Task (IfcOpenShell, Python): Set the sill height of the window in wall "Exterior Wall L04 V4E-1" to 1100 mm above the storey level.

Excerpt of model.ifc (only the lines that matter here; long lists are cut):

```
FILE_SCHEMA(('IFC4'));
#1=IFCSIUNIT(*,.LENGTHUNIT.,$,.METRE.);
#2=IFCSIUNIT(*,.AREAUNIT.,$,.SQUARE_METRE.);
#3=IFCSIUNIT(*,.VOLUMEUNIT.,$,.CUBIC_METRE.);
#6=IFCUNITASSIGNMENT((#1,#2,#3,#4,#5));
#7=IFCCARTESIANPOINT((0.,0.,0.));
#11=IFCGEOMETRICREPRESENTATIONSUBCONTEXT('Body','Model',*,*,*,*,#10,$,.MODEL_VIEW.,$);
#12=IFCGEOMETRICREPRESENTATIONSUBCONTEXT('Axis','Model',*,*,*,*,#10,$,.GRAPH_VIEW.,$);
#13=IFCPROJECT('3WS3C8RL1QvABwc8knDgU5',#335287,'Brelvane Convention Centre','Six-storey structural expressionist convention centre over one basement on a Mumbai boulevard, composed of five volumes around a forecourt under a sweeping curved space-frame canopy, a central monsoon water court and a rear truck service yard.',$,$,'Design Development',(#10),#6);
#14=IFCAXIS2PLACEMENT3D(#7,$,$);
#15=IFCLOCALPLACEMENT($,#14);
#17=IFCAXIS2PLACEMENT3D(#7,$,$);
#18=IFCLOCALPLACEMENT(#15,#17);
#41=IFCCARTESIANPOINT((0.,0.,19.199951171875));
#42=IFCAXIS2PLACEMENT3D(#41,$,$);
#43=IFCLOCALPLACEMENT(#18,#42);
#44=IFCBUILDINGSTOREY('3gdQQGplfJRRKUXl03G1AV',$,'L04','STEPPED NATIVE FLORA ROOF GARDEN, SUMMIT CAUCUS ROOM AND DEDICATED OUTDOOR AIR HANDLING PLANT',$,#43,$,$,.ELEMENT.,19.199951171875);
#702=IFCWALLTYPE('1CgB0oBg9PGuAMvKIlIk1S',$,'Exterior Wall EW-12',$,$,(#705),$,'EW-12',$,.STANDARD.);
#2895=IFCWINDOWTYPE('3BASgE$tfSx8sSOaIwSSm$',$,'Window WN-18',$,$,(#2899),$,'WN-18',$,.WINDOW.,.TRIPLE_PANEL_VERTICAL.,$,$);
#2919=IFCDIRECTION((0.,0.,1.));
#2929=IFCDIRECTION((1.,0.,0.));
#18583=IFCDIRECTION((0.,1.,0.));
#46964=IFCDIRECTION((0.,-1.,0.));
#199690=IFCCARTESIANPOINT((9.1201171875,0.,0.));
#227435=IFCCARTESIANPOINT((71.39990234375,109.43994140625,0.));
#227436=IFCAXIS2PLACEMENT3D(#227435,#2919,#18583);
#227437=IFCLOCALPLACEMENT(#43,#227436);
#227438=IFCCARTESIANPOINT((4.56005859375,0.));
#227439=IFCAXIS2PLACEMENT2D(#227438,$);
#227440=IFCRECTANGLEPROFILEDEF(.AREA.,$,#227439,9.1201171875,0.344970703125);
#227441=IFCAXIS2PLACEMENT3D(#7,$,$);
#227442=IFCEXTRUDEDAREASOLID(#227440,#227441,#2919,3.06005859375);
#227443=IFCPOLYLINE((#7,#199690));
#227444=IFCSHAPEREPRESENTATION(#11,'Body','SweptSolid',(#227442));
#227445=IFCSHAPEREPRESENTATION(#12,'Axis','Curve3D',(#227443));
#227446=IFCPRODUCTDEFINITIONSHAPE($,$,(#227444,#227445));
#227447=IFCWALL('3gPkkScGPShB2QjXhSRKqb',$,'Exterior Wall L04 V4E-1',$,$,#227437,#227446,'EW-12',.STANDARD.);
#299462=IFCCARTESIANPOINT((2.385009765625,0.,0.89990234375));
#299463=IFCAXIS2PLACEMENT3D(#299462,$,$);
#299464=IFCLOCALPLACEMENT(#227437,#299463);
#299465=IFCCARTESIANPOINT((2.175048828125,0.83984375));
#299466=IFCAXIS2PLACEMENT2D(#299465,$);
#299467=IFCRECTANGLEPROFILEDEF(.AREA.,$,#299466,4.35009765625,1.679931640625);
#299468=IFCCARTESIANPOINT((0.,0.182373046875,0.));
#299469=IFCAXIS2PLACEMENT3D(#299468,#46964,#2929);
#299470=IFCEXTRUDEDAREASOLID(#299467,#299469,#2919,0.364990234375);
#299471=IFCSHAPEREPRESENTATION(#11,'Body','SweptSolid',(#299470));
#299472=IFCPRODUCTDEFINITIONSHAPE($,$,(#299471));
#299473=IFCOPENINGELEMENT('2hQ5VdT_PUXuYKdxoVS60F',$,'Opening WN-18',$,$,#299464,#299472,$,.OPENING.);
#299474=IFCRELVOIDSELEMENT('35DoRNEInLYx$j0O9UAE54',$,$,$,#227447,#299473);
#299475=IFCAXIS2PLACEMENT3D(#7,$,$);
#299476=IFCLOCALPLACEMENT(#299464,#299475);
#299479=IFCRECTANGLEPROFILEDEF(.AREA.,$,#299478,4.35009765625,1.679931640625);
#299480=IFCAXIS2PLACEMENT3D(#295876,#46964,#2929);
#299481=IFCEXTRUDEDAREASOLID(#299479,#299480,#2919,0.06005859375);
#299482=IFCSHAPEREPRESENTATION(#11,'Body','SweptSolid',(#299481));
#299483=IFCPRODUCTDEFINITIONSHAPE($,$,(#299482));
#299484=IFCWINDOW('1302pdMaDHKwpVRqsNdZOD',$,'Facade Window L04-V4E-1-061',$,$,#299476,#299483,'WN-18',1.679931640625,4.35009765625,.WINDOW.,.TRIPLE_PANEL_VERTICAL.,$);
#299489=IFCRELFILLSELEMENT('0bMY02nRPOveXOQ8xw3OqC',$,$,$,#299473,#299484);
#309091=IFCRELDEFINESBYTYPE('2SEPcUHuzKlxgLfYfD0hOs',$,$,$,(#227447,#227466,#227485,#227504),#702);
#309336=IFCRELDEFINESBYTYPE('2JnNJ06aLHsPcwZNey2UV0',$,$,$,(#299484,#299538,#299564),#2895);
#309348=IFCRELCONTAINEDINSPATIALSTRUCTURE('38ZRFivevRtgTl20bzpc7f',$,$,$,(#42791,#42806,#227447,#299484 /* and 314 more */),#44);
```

```python
import numpy as np
import ifcopenshell
import ifcopenshell.api.geometry
import ifcopenshell.geom
import ifcopenshell.util.element
import ifcopenshell.util.placement
import ifcopenshell.util.shape
import ifcopenshell.util.unit

model = ifcopenshell.open("model.ifc")
unit_scale = ifcopenshell.util.unit.calculate_unit_scale(model)

window = model.by_id(299484)
opening = window.FillsVoids[0].RelatingOpeningElement
storey = ifcopenshell.util.element.get_container(window, ifc_class="IfcBuildingStorey")
level = ifcopenshell.util.placement.get_local_placement(storey.ObjectPlacement)[2, 3]

# The opening's origin need not be at the sill, so measure its lowest point.
shape = ifcopenshell.geom.create_shape(ifcopenshell.geom.settings(), opening)
bottom = ifcopenshell.util.shape.get_shape_bottom_elevation(shape, shape.geometry) / unit_scale
dz = level + 1.1 - bottom

shift = np.array([0.0, 0.0, dz])
# The window is placed relative to its opening, so it follows when the opening moves.
matrix = ifcopenshell.util.placement.get_local_placement(opening.ObjectPlacement)
matrix[:3, 3] += shift
ifcopenshell.api.geometry.edit_object_placement(
    model, product=opening, matrix=matrix, is_si=False, should_transform_children=True
)

print(f"moved by {dz * unit_scale:+.3f} m")

model.write("model_rev.ifc")
```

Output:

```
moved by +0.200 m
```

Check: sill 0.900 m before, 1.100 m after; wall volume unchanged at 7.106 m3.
